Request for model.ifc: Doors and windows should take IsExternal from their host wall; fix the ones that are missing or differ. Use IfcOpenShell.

First a look at what the model holds.

```python
import ifcopenshell
import ifcopenshell.util.element

model = ifcopenshell.open("model.ifc")
print(model.schema)
seen = {}
for e in model.by_type("IfcDoor") + model.by_type("IfcWindow"):
    if not e.FillsVoids:
        continue
    host = e.FillsVoids[0].RelatingOpeningElement.VoidsElements[0].RelatingBuildingElement
    own = ifcopenshell.util.element.get_pset(e, f"Pset_{e.is_a()[3:].removesuffix('StandardCase')}Common", "IsExternal")
    wall = ifcopenshell.util.element.get_pset(host, "Pset_WallCommon", "IsExternal")
    seen[e.is_a(), own, wall] = seen.get((e.is_a(), own, wall), 0) + 1
for (cls, own, wall), count in sorted(seen.items(), key=str):
    print(count, cls, "IsExternal:", own, "| host wall:", wall)
```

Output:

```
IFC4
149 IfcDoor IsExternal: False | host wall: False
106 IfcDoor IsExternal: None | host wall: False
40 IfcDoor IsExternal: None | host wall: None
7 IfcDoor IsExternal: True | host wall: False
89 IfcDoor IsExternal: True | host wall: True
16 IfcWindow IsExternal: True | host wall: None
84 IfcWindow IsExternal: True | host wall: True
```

```python
import ifcopenshell
import ifcopenshell.api.pset
import ifcopenshell.util.element

model = ifcopenshell.open("model.ifc")

count = 0
for ifc_class, pset_name in (("IfcDoor", "Pset_DoorCommon"), ("IfcWindow", "Pset_WindowCommon")):
    for e in model.by_type(ifc_class):
        if not e.FillsVoids:
            continue
        host = e.FillsVoids[0].RelatingOpeningElement.VoidsElements[0].RelatingBuildingElement
        external = ifcopenshell.util.element.get_pset(host, "Pset_WallCommon", "IsExternal")
        if external is None or ifcopenshell.util.element.get_pset(e, pset_name, "IsExternal") == external:
            continue
        pset = ifcopenshell.api.pset.add_pset(model, product=e, name=pset_name)
        ifcopenshell.api.pset.edit_pset(model, pset=pset, properties={"IsExternal": external})
        count += 1

print(count, "updated")

model.write("model_updated.ifc")
```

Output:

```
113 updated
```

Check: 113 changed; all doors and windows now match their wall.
